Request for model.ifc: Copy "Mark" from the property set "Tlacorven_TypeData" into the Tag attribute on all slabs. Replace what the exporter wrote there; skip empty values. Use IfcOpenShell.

First a look at what the model holds.

```python
import ifcopenshell
import ifcopenshell.util.element

model = ifcopenshell.open("model.ifc")
print(model.schema)
slabs = model.by_type("IfcSlab")
print(len(slabs), "slabs")
for e in slabs[:8]:
    source = ifcopenshell.util.element.get_pset(e, "Tlacorven_TypeData", "Mark")
    target = e.Tag
    print(e.id(), repr(source), repr(target), sep=" | ")
```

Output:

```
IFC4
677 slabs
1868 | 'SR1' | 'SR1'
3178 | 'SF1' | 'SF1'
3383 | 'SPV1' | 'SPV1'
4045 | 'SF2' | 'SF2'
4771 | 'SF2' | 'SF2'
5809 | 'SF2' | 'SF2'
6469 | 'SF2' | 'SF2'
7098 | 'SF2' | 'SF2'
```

```python
import ifcopenshell
import ifcopenshell.util.element

model = ifcopenshell.open("model.ifc")

count = 0
for e in model.by_type("IfcSlab"):
    value = ifcopenshell.util.element.get_pset(e, "Tlacorven_TypeData", "Mark")
    current = e.Tag
    if not value or not value.strip() or current == value:
        continue
    e.Tag = value
    count += 1

print(count, "slabs updated")

model.write("model_v2.ifc")
```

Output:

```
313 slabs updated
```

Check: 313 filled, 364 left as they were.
